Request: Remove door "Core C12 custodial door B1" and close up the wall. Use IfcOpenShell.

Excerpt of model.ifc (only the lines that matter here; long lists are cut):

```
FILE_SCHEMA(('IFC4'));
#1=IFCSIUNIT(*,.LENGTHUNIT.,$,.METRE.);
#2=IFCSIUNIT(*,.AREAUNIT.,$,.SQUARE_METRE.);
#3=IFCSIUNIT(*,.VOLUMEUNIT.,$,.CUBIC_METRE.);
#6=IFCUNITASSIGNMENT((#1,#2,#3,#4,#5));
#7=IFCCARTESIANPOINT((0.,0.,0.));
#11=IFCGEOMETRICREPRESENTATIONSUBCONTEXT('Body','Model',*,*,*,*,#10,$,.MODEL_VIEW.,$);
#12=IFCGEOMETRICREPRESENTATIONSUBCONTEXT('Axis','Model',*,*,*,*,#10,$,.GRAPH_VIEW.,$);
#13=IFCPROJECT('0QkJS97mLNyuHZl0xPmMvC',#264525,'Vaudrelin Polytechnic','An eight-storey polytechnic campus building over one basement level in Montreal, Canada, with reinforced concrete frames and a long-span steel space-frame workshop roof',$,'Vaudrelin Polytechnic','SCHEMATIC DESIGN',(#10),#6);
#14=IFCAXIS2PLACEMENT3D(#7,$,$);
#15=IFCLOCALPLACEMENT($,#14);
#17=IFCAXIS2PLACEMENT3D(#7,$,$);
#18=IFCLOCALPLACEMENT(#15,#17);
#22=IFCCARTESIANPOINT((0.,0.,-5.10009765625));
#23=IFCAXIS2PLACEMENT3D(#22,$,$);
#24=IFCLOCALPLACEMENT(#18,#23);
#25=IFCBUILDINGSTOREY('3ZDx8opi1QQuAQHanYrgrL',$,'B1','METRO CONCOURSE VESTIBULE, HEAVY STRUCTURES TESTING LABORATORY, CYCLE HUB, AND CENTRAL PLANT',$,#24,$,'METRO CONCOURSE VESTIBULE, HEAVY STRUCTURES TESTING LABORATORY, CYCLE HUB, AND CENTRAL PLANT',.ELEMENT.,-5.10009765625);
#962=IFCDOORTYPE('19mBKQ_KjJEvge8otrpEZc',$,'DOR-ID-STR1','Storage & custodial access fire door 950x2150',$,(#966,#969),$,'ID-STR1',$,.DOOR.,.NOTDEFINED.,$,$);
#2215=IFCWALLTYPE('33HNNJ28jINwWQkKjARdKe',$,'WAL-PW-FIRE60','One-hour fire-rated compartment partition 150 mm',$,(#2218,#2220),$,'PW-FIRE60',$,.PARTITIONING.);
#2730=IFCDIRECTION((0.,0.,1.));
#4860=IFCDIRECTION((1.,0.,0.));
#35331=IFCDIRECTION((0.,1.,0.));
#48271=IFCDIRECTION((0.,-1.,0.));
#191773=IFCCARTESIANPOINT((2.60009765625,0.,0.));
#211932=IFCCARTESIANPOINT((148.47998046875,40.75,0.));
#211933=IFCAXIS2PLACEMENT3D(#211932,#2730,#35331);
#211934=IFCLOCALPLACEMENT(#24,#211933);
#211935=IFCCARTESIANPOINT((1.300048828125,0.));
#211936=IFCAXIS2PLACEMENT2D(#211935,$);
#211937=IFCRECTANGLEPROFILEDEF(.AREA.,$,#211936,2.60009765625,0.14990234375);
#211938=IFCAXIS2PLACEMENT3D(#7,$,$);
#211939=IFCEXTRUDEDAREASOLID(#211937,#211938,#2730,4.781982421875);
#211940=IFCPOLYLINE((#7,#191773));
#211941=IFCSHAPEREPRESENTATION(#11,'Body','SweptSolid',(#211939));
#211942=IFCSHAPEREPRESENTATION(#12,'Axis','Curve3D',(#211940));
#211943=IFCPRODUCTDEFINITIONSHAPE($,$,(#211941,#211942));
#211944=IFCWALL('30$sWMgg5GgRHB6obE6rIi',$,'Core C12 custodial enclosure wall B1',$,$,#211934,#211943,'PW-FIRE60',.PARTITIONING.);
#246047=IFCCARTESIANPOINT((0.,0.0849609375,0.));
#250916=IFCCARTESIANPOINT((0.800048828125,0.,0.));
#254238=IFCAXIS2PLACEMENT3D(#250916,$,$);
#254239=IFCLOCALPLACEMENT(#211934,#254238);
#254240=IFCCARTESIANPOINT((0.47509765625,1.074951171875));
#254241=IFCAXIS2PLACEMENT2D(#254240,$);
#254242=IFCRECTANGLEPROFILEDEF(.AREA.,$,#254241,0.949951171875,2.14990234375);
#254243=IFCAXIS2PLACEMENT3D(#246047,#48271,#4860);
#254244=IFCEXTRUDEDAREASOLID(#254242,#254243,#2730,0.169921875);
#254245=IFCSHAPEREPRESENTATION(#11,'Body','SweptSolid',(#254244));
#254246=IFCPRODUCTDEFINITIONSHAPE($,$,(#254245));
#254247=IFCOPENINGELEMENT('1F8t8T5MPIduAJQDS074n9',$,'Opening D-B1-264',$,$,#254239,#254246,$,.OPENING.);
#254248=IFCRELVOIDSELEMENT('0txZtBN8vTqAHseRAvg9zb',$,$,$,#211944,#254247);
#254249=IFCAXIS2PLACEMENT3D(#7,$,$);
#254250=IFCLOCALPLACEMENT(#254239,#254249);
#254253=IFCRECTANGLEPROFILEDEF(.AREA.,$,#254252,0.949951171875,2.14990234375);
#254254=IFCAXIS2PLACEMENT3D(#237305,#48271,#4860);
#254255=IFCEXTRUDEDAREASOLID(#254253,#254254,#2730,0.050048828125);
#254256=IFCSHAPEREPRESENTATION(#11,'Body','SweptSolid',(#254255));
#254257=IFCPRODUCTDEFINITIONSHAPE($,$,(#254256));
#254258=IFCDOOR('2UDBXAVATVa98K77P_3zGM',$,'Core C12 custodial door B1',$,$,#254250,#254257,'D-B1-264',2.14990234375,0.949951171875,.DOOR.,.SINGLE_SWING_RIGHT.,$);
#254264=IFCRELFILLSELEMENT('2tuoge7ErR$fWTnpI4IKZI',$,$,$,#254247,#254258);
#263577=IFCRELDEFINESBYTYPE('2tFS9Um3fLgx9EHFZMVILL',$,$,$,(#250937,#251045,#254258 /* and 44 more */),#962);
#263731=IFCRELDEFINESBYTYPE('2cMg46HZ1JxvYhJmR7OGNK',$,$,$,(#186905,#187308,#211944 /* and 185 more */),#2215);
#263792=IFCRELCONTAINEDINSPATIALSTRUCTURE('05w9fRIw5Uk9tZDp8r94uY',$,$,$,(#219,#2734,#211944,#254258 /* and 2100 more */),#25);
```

```python
import ifcopenshell
import ifcopenshell.api.feature
import ifcopenshell.api.root
import ifcopenshell.geom
import ifcopenshell.util.shape

model = ifcopenshell.open("model.ifc")
settings = ifcopenshell.geom.settings()


def volume(element):
    """Net volume in cubic metres, openings subtracted."""
    shape = ifcopenshell.geom.create_shape(settings, element)
    return ifcopenshell.util.shape.get_volume(shape.geometry)


door = model.by_id(254258)
opening = door.FillsVoids[0].RelatingOpeningElement
wall = opening.VoidsElements[0].RelatingBuildingElement
before = volume(wall)

ifcopenshell.api.root.remove_product(model, product=door)
ifcopenshell.api.feature.remove_feature(model, feature=opening)

after = volume(wall)

print(f"wall volume {before:.3f} -> {after:.3f} m3")

model.write("model_updated.ifc")
```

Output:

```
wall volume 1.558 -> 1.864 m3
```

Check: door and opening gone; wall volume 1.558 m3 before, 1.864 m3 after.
